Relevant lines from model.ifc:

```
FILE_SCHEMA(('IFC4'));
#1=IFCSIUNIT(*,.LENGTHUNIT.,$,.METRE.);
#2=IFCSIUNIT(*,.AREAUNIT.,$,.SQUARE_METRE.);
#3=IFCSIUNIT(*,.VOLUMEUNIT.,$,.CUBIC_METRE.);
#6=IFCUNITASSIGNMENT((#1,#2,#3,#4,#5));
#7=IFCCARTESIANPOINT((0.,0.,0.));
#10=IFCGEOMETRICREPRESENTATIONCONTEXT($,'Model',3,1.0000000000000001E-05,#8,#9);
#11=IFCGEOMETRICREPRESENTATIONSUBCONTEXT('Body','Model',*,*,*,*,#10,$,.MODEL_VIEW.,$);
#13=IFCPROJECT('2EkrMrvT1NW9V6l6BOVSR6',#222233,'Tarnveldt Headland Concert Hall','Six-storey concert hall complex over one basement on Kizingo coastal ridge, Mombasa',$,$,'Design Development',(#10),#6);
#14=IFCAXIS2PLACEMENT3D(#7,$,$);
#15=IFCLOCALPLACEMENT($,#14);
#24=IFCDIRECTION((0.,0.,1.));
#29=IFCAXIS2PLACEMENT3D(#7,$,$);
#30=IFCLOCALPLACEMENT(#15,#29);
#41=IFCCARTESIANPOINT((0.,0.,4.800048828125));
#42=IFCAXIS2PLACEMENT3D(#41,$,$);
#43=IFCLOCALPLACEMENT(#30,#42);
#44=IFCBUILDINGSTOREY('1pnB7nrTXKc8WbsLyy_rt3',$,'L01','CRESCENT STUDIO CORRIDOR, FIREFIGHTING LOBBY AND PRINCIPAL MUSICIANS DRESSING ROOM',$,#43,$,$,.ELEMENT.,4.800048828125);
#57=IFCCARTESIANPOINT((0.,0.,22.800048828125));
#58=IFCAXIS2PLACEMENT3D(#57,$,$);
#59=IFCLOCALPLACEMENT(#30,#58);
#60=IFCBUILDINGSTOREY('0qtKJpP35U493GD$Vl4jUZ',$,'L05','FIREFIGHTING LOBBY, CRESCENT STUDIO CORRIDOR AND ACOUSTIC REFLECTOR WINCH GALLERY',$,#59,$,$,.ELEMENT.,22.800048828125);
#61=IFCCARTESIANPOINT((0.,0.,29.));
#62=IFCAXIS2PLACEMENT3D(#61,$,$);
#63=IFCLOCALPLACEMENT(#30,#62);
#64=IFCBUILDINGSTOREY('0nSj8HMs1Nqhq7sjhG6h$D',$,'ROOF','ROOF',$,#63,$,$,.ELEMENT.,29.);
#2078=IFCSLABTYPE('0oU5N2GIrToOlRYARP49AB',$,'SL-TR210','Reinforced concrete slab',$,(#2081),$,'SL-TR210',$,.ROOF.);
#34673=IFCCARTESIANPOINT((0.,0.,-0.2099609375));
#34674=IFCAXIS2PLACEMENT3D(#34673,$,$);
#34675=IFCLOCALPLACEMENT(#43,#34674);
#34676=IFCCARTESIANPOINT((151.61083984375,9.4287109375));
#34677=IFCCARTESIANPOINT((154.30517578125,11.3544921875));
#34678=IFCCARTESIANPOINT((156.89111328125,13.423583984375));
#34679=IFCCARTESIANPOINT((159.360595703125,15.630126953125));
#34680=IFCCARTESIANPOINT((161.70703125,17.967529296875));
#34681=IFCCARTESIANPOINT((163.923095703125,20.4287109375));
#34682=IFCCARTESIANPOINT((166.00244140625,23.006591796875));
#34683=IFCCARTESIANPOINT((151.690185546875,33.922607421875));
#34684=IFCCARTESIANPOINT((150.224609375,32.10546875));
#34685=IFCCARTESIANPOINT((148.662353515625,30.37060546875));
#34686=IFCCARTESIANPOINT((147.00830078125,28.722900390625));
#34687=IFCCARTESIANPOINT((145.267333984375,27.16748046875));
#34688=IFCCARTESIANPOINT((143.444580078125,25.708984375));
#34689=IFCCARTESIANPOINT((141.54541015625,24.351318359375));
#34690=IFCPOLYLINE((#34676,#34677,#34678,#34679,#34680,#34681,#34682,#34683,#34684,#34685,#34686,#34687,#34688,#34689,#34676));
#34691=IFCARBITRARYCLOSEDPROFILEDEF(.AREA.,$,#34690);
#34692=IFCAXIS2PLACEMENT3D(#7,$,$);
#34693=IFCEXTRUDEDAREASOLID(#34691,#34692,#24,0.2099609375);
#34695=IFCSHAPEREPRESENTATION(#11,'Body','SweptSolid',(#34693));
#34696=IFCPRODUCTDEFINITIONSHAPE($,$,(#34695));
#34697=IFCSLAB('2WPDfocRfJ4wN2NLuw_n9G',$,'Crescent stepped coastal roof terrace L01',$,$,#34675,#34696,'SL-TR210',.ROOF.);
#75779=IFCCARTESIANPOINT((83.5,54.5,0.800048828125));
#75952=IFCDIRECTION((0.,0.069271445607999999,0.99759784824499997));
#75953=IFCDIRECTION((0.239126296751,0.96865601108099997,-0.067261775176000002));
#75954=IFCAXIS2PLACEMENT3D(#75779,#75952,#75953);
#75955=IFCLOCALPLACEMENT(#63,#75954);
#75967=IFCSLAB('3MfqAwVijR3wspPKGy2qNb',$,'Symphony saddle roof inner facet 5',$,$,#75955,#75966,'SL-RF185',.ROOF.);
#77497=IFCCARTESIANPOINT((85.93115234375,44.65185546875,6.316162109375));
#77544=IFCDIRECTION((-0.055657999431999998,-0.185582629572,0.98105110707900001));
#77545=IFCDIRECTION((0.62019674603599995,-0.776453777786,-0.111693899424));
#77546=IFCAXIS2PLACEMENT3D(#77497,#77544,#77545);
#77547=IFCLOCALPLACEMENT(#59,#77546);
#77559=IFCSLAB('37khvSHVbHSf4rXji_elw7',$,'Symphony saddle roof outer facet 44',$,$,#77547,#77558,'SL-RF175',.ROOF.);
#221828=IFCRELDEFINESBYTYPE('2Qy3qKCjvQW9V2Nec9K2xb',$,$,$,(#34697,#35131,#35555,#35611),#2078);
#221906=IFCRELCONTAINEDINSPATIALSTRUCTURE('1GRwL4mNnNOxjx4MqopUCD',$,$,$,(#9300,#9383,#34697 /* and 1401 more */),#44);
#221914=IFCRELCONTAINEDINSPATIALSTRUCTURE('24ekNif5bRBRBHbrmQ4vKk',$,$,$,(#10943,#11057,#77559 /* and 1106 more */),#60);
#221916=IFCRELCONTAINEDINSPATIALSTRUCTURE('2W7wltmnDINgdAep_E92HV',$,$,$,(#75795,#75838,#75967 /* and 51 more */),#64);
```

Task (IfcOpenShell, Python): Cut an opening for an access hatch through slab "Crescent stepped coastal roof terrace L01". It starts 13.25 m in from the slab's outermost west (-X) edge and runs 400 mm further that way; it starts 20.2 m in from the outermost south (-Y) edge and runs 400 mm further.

```python
import numpy as np
import ifcopenshell
import ifcopenshell.api.feature
import ifcopenshell.api.geometry
import ifcopenshell.api.root
import ifcopenshell.geom
import ifcopenshell.util.placement
import ifcopenshell.util.representation
import ifcopenshell.util.shape
import ifcopenshell.util.unit

model = ifcopenshell.open("model.ifc")
unit_scale = ifcopenshell.util.unit.calculate_unit_scale(model)
settings = ifcopenshell.geom.settings()


def volume(element):
    """Net volume in cubic metres, openings subtracted."""
    shape = ifcopenshell.geom.create_shape(settings, element)
    return ifcopenshell.util.shape.get_volume(shape.geometry)


slab = model.by_guid("2WPDfocRfJ4wN2NLuw_n9G")
before = volume(slab)

# Extent in the slab's own axes, in metres. The edges named are its -X and -Y sides.
slab_shape = ifcopenshell.geom.create_shape(settings, slab)
vertices = ifcopenshell.util.shape.get_vertices(slab_shape.geometry)
x_min, y_min, bottom = vertices.min(axis=0)
top = vertices[:, 2].max()

opening = ifcopenshell.api.root.create_entity(model, ifc_class="IfcOpeningElement", name="Access hatch opening", predefined_type="OPENING")
context = ifcopenshell.util.representation.get_context(model, "Model", "Body", "MODEL_VIEW")
width, depth = 0.4, 0.4
outline = [(0.0, 0.0), (width, 0.0), (width, depth), (0.0, depth), (0.0, 0.0)]
# Overshoot both faces by 50 mm so the cut is clean.
shape = ifcopenshell.api.geometry.add_slab_representation(
    model, context=context, depth=top - bottom + 0.1, polyline=outline
)
ifcopenshell.api.geometry.assign_representation(model, product=opening, representation=shape)

matrix = ifcopenshell.util.placement.get_local_placement(slab.ObjectPlacement)
matrix[:, 3] = matrix @ np.append(np.array([x_min + 13.25, y_min + 20.2, bottom - 0.05]) / unit_scale, 1.0)
ifcopenshell.api.geometry.edit_object_placement(model, product=opening, matrix=matrix, is_si=False)
ifcopenshell.api.feature.add_feature(model, feature=opening, element=slab)

after = volume(slab)

print(f"slab volume {before:.3f} -> {after:.3f} m3")

model.write("model_v2.ifc")
```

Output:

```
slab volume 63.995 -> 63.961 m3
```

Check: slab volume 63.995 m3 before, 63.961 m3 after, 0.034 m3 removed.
